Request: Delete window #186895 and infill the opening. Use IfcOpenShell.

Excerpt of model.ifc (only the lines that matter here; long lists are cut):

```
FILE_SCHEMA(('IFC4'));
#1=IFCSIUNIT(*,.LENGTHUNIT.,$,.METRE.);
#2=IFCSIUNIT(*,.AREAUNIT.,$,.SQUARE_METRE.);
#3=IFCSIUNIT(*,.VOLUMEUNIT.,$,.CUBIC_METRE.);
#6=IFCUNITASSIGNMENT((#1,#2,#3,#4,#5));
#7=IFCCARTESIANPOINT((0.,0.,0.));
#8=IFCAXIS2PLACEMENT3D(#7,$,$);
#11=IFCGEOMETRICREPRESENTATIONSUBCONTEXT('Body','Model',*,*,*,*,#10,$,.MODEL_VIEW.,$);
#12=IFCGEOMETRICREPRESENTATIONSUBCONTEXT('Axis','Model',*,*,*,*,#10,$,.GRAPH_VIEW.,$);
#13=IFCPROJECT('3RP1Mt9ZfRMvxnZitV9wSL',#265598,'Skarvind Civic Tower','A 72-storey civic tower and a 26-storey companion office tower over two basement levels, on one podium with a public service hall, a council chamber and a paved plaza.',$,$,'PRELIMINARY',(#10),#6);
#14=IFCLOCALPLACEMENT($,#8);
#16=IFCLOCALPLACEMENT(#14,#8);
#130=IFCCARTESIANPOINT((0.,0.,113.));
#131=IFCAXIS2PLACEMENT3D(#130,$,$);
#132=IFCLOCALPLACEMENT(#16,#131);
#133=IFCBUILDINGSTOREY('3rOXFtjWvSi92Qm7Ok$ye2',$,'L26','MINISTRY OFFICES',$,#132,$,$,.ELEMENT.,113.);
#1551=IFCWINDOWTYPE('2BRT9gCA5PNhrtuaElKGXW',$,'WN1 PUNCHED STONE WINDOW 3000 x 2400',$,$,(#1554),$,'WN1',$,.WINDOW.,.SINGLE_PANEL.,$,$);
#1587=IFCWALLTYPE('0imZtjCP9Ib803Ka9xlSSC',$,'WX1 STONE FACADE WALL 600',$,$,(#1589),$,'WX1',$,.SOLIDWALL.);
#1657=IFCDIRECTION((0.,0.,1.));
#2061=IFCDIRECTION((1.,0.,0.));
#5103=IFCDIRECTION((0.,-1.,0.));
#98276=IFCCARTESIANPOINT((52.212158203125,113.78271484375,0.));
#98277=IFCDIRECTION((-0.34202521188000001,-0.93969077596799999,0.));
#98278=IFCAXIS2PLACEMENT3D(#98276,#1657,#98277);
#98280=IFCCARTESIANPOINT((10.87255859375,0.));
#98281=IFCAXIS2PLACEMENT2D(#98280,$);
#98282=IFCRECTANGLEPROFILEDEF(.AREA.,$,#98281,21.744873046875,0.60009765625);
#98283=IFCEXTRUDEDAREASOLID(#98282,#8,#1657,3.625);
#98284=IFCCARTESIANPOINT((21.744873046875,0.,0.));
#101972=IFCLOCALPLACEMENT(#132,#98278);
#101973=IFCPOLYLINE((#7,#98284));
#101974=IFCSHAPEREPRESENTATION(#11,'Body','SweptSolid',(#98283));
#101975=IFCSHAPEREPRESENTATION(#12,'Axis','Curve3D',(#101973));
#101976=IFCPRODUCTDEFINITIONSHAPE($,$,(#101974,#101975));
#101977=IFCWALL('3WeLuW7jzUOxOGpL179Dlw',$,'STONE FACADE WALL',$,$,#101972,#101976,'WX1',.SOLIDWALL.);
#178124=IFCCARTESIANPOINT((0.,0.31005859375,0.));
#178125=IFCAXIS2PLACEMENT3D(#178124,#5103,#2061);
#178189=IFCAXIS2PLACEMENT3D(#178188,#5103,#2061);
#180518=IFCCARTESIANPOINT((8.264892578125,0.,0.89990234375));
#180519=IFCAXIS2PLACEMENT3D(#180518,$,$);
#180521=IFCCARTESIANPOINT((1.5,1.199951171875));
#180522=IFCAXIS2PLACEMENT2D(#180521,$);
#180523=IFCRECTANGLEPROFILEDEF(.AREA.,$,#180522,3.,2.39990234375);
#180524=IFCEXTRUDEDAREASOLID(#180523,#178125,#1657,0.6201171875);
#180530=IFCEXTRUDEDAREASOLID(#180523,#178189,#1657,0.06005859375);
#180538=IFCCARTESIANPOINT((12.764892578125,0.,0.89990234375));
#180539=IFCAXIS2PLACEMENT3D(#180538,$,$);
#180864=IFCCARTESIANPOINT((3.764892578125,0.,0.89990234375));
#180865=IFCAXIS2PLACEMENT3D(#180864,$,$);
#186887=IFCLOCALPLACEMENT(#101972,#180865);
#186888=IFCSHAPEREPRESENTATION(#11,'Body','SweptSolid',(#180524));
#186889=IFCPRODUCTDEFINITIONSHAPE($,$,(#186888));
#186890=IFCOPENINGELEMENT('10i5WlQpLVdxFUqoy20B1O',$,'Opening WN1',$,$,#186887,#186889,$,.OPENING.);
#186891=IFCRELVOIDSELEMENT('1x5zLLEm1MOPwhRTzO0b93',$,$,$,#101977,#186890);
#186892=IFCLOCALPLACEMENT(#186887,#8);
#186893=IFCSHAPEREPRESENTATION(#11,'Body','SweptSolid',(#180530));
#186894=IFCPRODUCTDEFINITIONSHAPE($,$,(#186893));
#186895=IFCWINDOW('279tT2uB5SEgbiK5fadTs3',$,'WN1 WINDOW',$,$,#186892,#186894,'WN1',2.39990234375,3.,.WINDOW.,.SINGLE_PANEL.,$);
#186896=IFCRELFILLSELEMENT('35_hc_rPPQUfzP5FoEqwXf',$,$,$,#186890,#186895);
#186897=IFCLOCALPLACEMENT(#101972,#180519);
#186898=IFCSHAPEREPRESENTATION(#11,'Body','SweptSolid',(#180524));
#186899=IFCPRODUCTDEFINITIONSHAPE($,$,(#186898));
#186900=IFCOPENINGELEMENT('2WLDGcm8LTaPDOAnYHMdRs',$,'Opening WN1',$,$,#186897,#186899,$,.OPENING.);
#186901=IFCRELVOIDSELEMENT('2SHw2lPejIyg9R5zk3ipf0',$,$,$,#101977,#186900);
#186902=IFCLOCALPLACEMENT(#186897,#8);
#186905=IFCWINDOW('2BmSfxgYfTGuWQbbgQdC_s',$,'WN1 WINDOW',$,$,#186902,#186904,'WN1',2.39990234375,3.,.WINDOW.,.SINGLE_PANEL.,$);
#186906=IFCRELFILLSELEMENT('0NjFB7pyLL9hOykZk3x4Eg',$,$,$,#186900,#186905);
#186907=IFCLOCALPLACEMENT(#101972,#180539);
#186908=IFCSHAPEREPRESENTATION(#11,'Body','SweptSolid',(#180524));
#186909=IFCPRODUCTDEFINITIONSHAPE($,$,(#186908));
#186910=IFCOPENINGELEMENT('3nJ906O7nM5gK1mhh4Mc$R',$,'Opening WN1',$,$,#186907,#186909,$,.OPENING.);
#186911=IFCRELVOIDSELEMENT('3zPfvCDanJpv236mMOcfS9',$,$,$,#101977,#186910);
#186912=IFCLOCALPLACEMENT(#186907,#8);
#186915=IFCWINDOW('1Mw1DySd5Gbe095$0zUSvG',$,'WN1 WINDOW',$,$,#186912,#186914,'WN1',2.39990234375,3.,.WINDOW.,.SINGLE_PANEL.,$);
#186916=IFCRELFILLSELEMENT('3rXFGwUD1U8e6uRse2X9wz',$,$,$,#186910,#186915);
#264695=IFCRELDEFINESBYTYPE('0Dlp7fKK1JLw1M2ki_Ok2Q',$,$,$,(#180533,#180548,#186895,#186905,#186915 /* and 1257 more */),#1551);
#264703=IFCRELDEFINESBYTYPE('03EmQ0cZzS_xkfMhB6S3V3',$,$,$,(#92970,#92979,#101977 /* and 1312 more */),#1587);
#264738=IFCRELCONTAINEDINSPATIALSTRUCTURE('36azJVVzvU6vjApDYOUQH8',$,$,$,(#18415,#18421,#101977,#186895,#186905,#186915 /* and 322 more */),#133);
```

```python
import ifcopenshell
import ifcopenshell.api.feature
import ifcopenshell.api.root
import ifcopenshell.geom
import ifcopenshell.util.shape

model = ifcopenshell.open("model.ifc")
settings = ifcopenshell.geom.settings()


def volume(element):
    """Net volume in cubic metres, openings subtracted."""
    shape = ifcopenshell.geom.create_shape(settings, element)
    return ifcopenshell.util.shape.get_volume(shape.geometry)


window = model.by_guid("279tT2uB5SEgbiK5fadTs3")
opening = window.FillsVoids[0].RelatingOpeningElement
wall = opening.VoidsElements[0].RelatingBuildingElement
before = volume(wall)

ifcopenshell.api.root.remove_product(model, product=window)
ifcopenshell.api.feature.remove_feature(model, feature=opening)

after = volume(wall)

print(f"wall volume {before:.3f} -> {after:.3f} m3")

model.write("model_v2.ifc")
```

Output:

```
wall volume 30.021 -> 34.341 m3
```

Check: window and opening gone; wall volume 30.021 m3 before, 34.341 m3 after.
